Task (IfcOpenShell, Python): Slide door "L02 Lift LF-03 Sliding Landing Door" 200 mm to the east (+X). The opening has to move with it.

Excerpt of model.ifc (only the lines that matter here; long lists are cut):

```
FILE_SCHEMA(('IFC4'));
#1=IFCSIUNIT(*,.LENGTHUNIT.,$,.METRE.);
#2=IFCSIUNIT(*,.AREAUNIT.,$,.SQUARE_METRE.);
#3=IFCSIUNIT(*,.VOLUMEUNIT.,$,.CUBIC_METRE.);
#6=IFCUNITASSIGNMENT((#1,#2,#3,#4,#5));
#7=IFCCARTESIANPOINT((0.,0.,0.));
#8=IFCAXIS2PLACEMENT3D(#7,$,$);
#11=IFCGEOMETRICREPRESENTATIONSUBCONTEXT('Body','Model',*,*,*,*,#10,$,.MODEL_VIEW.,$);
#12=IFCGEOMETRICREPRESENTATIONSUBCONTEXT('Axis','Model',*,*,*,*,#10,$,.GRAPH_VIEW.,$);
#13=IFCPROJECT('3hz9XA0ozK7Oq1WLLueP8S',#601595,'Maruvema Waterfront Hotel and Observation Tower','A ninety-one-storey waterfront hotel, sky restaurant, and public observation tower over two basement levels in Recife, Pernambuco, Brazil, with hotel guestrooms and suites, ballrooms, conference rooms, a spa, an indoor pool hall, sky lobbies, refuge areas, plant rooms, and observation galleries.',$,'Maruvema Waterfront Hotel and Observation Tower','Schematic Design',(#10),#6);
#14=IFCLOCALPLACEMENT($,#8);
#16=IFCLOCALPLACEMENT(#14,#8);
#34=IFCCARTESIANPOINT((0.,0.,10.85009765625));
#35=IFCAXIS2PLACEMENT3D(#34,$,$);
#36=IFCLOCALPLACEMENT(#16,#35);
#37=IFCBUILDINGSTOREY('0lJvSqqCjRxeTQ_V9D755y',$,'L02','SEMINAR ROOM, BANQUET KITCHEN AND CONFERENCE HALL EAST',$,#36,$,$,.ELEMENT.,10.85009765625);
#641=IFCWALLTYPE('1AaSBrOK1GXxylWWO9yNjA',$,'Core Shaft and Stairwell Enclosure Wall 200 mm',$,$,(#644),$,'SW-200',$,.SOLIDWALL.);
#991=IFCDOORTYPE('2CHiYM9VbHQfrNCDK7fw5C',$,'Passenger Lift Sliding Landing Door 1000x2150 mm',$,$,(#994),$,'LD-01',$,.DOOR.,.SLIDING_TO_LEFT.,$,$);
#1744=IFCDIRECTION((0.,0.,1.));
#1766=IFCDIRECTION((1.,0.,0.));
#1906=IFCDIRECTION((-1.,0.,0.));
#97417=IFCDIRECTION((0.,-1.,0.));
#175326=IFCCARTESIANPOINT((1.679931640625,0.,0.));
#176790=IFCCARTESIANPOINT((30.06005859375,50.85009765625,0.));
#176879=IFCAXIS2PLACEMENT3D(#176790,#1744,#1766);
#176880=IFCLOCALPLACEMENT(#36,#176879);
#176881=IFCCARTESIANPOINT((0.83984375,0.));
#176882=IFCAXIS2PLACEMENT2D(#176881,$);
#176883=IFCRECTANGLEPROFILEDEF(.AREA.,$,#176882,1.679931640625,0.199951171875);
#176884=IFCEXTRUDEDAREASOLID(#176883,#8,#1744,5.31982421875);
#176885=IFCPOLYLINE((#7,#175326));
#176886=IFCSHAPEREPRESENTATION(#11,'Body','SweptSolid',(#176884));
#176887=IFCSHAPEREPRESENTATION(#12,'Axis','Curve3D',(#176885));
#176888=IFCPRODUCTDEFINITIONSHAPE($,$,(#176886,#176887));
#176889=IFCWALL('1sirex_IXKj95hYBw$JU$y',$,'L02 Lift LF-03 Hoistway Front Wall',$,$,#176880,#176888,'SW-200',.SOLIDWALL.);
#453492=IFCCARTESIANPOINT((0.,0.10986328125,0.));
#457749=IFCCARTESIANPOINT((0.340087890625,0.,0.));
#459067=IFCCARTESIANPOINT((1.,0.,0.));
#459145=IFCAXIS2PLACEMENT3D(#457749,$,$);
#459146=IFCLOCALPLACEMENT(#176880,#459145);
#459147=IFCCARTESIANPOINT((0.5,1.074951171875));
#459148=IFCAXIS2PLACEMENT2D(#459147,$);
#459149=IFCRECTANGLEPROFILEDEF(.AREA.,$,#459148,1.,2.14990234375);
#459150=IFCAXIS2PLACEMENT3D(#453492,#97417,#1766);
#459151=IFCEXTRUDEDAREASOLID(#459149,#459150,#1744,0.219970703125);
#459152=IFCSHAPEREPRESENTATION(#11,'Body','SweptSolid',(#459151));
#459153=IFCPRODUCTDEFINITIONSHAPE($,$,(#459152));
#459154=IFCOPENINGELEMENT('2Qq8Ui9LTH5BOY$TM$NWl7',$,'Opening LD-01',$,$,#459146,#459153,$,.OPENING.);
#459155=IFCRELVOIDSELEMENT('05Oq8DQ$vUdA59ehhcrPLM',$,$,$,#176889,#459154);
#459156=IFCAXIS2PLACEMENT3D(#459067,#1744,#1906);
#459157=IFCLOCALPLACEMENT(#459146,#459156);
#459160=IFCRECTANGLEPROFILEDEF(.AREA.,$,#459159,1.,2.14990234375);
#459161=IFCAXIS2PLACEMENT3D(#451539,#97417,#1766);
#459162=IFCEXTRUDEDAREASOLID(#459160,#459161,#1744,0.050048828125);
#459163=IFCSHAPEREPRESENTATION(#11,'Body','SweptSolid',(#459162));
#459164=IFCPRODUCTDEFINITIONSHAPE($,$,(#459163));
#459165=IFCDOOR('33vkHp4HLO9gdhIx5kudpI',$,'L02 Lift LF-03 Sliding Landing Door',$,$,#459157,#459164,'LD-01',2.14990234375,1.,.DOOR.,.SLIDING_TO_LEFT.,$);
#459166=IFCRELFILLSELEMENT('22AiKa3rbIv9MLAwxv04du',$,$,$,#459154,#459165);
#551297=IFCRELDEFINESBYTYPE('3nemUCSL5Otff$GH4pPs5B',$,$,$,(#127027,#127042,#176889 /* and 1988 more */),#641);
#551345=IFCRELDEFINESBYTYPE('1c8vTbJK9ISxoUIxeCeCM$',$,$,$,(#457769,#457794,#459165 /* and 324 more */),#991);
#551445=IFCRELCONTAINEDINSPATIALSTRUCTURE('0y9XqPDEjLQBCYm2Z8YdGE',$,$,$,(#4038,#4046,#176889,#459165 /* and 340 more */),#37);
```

```python
import ifcopenshell
import ifcopenshell.api.geometry
import ifcopenshell.util.placement
import ifcopenshell.util.unit

model = ifcopenshell.open("model.ifc")
unit_scale = ifcopenshell.util.unit.calculate_unit_scale(model)

door = model.by_id(459165)
opening = door.FillsVoids[0].RelatingOpeningElement
wall = opening.VoidsElements[0].RelatingBuildingElement

wall_matrix = ifcopenshell.util.placement.get_local_placement(wall.ObjectPlacement)
shift = wall_matrix[:3, 0] * 0.2 / unit_scale
before = ifcopenshell.util.placement.get_local_placement(door.ObjectPlacement)[:3, 3].copy()

# The door is placed relative to its opening, so it follows when the opening moves.
matrix = ifcopenshell.util.placement.get_local_placement(opening.ObjectPlacement)
matrix[:3, 3] += shift
ifcopenshell.api.geometry.edit_object_placement(
    model, product=opening, matrix=matrix, is_si=False, should_transform_children=True
)

after = ifcopenshell.util.placement.get_local_placement(door.ObjectPlacement)[:3, 3]
print("door moved by", (after - before).round(3) + 0.0)

model.write("model-out.ifc")
```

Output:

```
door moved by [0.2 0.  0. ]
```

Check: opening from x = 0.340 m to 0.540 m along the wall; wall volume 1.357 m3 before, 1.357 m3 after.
